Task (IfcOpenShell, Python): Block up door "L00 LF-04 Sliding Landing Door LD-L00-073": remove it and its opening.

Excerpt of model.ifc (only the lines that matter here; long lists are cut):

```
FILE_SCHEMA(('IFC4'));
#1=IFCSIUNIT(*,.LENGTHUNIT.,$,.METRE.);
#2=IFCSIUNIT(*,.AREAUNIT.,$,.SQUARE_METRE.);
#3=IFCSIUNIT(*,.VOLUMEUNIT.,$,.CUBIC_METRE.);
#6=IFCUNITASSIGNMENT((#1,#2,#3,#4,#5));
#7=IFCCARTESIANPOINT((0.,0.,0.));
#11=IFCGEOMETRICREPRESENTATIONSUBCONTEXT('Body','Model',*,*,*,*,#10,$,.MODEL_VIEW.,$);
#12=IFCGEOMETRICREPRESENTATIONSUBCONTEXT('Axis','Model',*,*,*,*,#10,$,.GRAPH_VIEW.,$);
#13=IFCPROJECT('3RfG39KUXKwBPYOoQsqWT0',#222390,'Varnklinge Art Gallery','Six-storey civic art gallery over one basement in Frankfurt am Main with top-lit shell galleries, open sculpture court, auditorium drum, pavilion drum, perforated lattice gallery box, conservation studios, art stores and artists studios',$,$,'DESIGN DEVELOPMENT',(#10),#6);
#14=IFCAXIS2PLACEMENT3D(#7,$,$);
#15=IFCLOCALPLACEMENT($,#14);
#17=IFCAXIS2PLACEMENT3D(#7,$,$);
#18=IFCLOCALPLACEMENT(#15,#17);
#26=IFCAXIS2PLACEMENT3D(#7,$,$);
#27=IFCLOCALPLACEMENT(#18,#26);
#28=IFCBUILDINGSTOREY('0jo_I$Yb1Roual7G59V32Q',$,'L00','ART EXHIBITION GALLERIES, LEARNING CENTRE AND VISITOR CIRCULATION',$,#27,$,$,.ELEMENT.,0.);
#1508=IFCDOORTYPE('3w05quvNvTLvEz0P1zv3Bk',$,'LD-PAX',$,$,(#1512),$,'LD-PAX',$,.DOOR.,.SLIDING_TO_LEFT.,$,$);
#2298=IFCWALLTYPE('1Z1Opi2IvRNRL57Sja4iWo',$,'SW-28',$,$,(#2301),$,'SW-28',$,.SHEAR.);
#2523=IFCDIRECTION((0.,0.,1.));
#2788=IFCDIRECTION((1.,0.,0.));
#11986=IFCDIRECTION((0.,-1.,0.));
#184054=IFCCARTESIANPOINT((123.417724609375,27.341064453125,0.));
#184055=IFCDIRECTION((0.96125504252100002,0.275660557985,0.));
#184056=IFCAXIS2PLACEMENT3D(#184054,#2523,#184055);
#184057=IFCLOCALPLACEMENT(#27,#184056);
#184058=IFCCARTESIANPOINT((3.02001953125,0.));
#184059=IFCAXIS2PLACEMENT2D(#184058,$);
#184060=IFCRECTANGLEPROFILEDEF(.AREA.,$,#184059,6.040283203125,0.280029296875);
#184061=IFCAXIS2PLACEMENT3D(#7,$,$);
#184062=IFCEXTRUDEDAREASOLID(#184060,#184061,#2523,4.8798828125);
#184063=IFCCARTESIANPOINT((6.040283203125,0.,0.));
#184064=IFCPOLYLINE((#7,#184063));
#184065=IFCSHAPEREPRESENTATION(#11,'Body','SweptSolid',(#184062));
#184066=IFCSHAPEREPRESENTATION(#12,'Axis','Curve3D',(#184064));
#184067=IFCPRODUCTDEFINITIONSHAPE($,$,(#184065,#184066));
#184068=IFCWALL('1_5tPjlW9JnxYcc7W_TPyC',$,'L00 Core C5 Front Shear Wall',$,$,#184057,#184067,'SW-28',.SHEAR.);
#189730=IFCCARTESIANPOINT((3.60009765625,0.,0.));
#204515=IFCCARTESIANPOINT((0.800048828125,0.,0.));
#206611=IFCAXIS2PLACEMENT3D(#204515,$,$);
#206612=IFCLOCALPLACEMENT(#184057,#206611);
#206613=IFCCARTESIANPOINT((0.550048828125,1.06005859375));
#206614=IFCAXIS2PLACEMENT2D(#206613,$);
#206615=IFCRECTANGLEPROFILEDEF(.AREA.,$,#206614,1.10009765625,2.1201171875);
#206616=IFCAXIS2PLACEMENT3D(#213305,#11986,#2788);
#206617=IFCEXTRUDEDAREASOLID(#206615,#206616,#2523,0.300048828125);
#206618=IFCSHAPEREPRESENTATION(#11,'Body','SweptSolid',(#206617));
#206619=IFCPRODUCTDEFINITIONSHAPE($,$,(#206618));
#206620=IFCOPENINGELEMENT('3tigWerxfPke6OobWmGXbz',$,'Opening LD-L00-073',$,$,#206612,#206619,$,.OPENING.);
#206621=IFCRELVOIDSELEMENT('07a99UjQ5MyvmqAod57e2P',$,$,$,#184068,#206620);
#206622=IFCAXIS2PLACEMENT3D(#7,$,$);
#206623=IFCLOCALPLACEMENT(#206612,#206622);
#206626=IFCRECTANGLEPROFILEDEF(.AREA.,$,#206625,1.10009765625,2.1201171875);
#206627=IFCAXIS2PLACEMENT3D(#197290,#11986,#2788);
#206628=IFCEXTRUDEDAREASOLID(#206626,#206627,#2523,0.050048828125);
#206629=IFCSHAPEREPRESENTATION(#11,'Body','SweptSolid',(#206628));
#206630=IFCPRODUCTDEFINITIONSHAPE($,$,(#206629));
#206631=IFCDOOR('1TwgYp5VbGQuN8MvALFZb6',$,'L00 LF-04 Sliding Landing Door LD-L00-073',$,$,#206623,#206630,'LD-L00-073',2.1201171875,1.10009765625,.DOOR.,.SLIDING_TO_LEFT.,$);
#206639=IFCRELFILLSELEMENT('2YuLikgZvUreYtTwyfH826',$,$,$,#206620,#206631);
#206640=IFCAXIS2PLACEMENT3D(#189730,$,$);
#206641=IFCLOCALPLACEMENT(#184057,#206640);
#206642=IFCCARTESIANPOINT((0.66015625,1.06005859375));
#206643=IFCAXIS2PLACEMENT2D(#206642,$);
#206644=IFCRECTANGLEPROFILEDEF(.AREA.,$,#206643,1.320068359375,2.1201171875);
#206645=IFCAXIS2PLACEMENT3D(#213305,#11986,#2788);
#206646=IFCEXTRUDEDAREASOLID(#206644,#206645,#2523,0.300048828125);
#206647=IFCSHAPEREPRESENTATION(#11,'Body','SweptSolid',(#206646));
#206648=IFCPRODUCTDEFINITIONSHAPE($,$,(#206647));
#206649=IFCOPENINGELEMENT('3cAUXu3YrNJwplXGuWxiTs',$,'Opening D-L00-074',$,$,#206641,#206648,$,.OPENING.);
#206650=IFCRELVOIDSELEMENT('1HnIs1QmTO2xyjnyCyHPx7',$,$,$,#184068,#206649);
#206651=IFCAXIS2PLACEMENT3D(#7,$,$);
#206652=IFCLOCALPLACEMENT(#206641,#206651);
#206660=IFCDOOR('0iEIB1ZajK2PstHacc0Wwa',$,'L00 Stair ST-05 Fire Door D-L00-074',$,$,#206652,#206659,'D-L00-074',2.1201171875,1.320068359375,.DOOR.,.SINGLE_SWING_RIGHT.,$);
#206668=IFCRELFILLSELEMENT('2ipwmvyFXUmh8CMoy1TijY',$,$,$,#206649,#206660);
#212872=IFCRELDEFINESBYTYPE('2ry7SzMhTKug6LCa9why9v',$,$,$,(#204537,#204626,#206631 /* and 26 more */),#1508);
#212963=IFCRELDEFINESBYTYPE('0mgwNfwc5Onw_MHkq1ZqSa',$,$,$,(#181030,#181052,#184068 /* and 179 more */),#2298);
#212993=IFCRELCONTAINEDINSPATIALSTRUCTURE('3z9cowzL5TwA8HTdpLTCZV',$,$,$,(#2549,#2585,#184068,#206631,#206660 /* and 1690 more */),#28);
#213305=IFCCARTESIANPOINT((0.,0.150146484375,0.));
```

```python
import ifcopenshell
import ifcopenshell.api.feature
import ifcopenshell.api.root
import ifcopenshell.geom
import ifcopenshell.util.shape

model = ifcopenshell.open("model.ifc")
settings = ifcopenshell.geom.settings()


def volume(element):
    """Net volume in cubic metres, openings subtracted."""
    shape = ifcopenshell.geom.create_shape(settings, element)
    return ifcopenshell.util.shape.get_volume(shape.geometry)


door = model.by_guid("1TwgYp5VbGQuN8MvALFZb6")
opening = door.FillsVoids[0].RelatingOpeningElement
wall = opening.VoidsElements[0].RelatingBuildingElement
before = volume(wall)

ifcopenshell.api.root.remove_product(model, product=door)
ifcopenshell.api.feature.remove_feature(model, feature=opening)

after = volume(wall)

print(f"wall volume {before:.3f} -> {after:.3f} m3")

model.write("model_edited.ifc")
```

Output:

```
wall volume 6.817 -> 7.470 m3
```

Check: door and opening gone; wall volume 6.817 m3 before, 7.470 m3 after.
